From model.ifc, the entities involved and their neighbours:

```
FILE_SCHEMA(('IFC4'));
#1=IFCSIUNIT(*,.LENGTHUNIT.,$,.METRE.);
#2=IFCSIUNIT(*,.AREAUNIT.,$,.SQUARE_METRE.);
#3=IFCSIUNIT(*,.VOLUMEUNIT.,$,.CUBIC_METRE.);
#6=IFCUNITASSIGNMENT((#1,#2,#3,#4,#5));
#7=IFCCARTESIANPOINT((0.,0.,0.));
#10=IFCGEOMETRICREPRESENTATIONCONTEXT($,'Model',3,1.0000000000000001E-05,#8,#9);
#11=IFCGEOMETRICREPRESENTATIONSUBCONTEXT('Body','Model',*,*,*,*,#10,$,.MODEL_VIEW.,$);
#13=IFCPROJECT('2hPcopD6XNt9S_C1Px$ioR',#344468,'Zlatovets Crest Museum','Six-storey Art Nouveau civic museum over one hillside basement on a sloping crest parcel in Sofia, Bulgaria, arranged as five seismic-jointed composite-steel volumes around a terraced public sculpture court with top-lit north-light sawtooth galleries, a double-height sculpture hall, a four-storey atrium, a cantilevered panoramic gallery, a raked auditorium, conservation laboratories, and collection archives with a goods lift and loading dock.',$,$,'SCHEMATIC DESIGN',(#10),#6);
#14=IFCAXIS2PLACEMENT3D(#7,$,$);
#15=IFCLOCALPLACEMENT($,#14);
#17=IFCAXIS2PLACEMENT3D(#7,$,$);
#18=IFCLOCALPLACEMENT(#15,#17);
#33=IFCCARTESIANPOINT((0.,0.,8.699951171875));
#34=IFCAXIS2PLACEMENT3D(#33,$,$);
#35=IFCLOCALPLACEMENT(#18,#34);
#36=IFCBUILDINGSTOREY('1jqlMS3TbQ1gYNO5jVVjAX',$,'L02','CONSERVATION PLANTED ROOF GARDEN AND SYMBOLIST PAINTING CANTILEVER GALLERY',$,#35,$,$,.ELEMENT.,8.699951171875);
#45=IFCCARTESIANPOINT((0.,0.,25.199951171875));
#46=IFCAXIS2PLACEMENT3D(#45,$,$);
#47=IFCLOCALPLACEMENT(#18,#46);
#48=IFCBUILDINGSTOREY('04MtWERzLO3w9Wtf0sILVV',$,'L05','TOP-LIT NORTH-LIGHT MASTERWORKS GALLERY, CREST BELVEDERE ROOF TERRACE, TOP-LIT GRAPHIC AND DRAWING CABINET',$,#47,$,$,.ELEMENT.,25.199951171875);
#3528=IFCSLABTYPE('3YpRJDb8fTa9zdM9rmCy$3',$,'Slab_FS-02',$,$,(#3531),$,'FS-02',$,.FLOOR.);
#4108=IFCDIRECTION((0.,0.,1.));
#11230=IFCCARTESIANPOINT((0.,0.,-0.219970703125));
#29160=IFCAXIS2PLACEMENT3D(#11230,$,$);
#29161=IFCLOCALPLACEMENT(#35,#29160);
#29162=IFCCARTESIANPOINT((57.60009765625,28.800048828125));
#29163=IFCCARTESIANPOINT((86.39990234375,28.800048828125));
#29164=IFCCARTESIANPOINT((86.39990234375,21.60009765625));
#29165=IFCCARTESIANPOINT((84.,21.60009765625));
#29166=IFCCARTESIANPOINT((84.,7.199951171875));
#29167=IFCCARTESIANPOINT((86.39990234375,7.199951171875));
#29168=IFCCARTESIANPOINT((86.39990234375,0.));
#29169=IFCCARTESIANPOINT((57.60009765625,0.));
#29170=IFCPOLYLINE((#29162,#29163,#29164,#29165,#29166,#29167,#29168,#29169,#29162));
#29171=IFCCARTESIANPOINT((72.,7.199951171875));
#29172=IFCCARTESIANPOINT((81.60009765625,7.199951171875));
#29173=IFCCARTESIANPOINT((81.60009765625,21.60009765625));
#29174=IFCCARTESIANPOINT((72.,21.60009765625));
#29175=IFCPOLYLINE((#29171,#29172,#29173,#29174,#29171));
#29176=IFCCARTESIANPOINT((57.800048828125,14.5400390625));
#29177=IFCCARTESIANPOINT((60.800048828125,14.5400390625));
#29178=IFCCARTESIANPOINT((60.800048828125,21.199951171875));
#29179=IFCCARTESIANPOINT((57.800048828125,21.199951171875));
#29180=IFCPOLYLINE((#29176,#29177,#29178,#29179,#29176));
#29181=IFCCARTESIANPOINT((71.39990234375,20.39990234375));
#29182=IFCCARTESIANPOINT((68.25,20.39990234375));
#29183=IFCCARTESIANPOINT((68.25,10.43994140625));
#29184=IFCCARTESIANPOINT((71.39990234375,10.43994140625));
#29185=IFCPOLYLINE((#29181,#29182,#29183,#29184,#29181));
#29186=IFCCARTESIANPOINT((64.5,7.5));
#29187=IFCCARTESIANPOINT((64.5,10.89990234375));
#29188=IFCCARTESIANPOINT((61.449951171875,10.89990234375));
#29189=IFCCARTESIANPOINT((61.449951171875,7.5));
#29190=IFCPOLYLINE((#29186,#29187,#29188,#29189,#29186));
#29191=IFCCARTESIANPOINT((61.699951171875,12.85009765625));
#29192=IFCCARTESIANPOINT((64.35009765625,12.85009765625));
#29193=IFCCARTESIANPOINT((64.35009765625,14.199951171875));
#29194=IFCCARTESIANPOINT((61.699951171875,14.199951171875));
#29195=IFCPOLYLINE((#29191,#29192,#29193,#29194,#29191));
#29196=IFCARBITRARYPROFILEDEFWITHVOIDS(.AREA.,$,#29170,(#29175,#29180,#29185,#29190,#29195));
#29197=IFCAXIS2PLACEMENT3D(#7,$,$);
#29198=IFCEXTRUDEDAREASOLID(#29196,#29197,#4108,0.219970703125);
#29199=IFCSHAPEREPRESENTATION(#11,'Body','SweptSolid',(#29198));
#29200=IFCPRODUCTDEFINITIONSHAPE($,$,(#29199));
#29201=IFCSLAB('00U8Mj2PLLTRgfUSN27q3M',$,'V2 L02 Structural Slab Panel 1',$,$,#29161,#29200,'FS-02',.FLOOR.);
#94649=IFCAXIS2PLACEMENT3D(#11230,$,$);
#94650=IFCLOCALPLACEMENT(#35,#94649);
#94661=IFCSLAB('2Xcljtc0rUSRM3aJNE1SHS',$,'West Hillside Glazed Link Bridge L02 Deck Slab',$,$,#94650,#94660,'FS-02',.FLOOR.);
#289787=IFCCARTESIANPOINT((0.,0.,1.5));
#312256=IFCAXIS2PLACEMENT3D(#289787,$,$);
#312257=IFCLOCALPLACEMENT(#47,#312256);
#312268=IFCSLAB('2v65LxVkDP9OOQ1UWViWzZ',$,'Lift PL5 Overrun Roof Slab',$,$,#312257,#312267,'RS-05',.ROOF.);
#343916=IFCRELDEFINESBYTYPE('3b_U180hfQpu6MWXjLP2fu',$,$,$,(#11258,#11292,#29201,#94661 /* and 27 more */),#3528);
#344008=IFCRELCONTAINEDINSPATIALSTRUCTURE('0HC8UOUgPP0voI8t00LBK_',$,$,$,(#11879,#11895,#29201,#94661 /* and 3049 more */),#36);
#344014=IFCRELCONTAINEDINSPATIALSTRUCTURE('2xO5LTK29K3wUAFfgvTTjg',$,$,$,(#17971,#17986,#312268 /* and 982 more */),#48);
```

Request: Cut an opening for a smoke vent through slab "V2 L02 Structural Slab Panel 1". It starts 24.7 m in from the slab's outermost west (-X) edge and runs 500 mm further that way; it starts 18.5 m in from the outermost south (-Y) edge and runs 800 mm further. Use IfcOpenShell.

```python
import numpy as np
import ifcopenshell
import ifcopenshell.api.feature
import ifcopenshell.api.geometry
import ifcopenshell.api.root
import ifcopenshell.geom
import ifcopenshell.util.placement
import ifcopenshell.util.representation
import ifcopenshell.util.shape
import ifcopenshell.util.unit

model = ifcopenshell.open("model.ifc")
unit_scale = ifcopenshell.util.unit.calculate_unit_scale(model)
settings = ifcopenshell.geom.settings()


def volume(element):
    """Net volume in cubic metres, openings subtracted."""
    shape = ifcopenshell.geom.create_shape(settings, element)
    return ifcopenshell.util.shape.get_volume(shape.geometry)


slab = model.by_id(29201)
before = volume(slab)

# Extent in the slab's own axes, in metres. The edges named are its -X and -Y sides.
slab_shape = ifcopenshell.geom.create_shape(settings, slab)
vertices = ifcopenshell.util.shape.get_vertices(slab_shape.geometry)
x_min, y_min, bottom = vertices.min(axis=0)
top = vertices[:, 2].max()

opening = ifcopenshell.api.root.create_entity(model, ifc_class="IfcOpeningElement", name="Smoke vent opening", predefined_type="OPENING")
context = ifcopenshell.util.representation.get_context(model, "Model", "Body", "MODEL_VIEW")
width, depth = 0.5, 0.8
outline = [(0.0, 0.0), (width, 0.0), (width, depth), (0.0, depth), (0.0, 0.0)]
# Overshoot both faces by 50 mm so the cut is clean.
shape = ifcopenshell.api.geometry.add_slab_representation(
    model, context=context, depth=top - bottom + 0.1, polyline=outline
)
ifcopenshell.api.geometry.assign_representation(model, product=opening, representation=shape)

matrix = ifcopenshell.util.placement.get_local_placement(slab.ObjectPlacement)
matrix[:, 3] = matrix @ np.append(np.array([x_min + 24.7, y_min + 18.5, bottom - 0.05]) / unit_scale, 1.0)
ifcopenshell.api.geometry.edit_object_placement(model, product=opening, matrix=matrix, is_si=False)
ifcopenshell.api.feature.add_feature(model, feature=opening, element=slab)

after = volume(slab)

print(f"slab volume {before:.3f} -> {after:.3f} m3")

model.write("model_rev.ifc")
```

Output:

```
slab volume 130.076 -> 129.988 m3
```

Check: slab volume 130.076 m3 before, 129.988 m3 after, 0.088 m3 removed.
